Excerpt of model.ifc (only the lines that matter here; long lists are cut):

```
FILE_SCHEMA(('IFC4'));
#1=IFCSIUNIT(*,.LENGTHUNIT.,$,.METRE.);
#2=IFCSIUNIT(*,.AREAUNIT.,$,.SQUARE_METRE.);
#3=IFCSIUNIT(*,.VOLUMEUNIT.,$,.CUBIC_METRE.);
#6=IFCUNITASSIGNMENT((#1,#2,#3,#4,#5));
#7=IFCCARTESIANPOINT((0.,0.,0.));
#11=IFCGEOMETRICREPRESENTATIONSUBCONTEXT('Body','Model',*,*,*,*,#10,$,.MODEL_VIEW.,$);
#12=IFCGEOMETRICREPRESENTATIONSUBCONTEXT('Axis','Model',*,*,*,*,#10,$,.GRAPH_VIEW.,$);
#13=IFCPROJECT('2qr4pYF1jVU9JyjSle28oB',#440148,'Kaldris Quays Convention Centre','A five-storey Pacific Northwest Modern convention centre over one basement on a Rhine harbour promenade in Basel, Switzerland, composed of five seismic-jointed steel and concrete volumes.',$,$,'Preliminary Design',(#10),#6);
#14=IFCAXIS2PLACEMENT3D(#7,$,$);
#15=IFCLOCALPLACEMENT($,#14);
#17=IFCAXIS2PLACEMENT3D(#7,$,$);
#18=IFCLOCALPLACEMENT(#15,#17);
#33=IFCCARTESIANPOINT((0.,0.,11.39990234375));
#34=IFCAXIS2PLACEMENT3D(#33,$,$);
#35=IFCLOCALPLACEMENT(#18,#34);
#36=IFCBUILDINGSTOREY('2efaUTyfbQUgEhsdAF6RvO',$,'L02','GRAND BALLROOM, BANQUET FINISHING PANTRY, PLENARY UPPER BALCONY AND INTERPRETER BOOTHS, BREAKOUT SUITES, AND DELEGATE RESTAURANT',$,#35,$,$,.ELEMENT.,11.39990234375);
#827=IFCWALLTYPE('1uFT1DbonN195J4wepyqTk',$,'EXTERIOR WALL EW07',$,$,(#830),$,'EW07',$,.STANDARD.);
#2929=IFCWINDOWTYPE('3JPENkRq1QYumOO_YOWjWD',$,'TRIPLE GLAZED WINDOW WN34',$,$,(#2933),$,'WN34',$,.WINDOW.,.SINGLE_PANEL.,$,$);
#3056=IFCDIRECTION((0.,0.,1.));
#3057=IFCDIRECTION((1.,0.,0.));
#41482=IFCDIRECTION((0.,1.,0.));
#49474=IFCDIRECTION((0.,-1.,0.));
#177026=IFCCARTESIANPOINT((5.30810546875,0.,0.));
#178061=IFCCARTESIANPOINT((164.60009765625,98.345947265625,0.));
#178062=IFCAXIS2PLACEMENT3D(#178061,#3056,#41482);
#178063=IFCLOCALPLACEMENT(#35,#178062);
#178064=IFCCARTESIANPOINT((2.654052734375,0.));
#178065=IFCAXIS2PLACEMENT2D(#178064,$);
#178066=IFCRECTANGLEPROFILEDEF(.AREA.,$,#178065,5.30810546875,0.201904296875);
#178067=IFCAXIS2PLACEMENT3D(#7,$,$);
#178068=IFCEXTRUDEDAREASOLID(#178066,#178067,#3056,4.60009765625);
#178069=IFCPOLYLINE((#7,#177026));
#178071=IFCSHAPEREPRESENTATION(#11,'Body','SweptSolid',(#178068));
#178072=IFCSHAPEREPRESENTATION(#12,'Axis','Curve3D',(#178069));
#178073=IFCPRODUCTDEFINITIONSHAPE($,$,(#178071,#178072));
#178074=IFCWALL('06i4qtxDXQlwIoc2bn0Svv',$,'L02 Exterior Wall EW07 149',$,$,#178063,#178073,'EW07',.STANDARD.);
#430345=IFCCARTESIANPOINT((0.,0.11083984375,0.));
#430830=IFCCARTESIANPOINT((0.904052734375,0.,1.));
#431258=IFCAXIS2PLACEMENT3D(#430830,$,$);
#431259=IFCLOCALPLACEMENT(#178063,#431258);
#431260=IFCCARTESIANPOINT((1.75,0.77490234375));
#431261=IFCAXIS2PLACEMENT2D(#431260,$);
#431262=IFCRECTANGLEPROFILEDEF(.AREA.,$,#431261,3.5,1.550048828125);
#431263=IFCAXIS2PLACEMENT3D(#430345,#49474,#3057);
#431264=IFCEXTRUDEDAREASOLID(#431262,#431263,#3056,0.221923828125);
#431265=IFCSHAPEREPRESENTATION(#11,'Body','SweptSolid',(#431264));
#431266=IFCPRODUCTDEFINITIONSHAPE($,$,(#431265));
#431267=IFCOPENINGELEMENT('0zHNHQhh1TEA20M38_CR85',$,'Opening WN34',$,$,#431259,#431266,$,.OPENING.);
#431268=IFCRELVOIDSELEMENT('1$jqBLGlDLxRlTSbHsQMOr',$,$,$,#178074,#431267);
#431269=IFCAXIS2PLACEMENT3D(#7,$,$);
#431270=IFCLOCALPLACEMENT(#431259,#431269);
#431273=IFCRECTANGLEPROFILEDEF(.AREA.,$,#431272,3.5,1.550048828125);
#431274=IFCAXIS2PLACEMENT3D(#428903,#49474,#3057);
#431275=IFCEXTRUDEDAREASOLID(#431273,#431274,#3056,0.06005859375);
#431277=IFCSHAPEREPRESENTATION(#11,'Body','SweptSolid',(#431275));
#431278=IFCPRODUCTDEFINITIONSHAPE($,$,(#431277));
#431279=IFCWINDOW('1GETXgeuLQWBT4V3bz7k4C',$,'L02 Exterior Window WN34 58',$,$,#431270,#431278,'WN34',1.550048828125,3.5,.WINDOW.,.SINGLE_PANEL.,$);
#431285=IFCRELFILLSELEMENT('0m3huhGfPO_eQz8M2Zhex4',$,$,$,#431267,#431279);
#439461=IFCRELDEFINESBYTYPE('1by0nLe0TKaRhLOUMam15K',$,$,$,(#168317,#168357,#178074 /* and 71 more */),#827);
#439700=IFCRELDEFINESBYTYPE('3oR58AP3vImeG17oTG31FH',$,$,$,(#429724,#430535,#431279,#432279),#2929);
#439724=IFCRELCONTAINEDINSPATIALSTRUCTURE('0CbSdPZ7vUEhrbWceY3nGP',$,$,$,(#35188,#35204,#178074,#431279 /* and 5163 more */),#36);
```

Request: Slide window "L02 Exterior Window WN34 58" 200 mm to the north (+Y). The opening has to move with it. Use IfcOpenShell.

```python
import ifcopenshell
import ifcopenshell.api.geometry
import ifcopenshell.util.placement

model = ifcopenshell.open("model.ifc")

window = model.by_guid("1GETXgeuLQWBT4V3bz7k4C")
opening = window.FillsVoids[0].RelatingOpeningElement
wall = opening.VoidsElements[0].RelatingBuildingElement

wall_matrix = ifcopenshell.util.placement.get_local_placement(wall.ObjectPlacement)
shift = wall_matrix[:3, 0] * 0.2
before = ifcopenshell.util.placement.get_local_placement(window.ObjectPlacement)[:3, 3].copy()

# The window is placed relative to its opening, so it follows when the opening moves.
matrix = ifcopenshell.util.placement.get_local_placement(opening.ObjectPlacement)
matrix[:3, 3] += shift
ifcopenshell.api.geometry.edit_object_placement(
    model, product=opening, matrix=matrix, is_si=False, should_transform_children=True
)

after = ifcopenshell.util.placement.get_local_placement(window.ObjectPlacement)[:3, 3]
print("window moved by", (after - before).round(3) + 0.0)

model.write("model_updated.ifc")
```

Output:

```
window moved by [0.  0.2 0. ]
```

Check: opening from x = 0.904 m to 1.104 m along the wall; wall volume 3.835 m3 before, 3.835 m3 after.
